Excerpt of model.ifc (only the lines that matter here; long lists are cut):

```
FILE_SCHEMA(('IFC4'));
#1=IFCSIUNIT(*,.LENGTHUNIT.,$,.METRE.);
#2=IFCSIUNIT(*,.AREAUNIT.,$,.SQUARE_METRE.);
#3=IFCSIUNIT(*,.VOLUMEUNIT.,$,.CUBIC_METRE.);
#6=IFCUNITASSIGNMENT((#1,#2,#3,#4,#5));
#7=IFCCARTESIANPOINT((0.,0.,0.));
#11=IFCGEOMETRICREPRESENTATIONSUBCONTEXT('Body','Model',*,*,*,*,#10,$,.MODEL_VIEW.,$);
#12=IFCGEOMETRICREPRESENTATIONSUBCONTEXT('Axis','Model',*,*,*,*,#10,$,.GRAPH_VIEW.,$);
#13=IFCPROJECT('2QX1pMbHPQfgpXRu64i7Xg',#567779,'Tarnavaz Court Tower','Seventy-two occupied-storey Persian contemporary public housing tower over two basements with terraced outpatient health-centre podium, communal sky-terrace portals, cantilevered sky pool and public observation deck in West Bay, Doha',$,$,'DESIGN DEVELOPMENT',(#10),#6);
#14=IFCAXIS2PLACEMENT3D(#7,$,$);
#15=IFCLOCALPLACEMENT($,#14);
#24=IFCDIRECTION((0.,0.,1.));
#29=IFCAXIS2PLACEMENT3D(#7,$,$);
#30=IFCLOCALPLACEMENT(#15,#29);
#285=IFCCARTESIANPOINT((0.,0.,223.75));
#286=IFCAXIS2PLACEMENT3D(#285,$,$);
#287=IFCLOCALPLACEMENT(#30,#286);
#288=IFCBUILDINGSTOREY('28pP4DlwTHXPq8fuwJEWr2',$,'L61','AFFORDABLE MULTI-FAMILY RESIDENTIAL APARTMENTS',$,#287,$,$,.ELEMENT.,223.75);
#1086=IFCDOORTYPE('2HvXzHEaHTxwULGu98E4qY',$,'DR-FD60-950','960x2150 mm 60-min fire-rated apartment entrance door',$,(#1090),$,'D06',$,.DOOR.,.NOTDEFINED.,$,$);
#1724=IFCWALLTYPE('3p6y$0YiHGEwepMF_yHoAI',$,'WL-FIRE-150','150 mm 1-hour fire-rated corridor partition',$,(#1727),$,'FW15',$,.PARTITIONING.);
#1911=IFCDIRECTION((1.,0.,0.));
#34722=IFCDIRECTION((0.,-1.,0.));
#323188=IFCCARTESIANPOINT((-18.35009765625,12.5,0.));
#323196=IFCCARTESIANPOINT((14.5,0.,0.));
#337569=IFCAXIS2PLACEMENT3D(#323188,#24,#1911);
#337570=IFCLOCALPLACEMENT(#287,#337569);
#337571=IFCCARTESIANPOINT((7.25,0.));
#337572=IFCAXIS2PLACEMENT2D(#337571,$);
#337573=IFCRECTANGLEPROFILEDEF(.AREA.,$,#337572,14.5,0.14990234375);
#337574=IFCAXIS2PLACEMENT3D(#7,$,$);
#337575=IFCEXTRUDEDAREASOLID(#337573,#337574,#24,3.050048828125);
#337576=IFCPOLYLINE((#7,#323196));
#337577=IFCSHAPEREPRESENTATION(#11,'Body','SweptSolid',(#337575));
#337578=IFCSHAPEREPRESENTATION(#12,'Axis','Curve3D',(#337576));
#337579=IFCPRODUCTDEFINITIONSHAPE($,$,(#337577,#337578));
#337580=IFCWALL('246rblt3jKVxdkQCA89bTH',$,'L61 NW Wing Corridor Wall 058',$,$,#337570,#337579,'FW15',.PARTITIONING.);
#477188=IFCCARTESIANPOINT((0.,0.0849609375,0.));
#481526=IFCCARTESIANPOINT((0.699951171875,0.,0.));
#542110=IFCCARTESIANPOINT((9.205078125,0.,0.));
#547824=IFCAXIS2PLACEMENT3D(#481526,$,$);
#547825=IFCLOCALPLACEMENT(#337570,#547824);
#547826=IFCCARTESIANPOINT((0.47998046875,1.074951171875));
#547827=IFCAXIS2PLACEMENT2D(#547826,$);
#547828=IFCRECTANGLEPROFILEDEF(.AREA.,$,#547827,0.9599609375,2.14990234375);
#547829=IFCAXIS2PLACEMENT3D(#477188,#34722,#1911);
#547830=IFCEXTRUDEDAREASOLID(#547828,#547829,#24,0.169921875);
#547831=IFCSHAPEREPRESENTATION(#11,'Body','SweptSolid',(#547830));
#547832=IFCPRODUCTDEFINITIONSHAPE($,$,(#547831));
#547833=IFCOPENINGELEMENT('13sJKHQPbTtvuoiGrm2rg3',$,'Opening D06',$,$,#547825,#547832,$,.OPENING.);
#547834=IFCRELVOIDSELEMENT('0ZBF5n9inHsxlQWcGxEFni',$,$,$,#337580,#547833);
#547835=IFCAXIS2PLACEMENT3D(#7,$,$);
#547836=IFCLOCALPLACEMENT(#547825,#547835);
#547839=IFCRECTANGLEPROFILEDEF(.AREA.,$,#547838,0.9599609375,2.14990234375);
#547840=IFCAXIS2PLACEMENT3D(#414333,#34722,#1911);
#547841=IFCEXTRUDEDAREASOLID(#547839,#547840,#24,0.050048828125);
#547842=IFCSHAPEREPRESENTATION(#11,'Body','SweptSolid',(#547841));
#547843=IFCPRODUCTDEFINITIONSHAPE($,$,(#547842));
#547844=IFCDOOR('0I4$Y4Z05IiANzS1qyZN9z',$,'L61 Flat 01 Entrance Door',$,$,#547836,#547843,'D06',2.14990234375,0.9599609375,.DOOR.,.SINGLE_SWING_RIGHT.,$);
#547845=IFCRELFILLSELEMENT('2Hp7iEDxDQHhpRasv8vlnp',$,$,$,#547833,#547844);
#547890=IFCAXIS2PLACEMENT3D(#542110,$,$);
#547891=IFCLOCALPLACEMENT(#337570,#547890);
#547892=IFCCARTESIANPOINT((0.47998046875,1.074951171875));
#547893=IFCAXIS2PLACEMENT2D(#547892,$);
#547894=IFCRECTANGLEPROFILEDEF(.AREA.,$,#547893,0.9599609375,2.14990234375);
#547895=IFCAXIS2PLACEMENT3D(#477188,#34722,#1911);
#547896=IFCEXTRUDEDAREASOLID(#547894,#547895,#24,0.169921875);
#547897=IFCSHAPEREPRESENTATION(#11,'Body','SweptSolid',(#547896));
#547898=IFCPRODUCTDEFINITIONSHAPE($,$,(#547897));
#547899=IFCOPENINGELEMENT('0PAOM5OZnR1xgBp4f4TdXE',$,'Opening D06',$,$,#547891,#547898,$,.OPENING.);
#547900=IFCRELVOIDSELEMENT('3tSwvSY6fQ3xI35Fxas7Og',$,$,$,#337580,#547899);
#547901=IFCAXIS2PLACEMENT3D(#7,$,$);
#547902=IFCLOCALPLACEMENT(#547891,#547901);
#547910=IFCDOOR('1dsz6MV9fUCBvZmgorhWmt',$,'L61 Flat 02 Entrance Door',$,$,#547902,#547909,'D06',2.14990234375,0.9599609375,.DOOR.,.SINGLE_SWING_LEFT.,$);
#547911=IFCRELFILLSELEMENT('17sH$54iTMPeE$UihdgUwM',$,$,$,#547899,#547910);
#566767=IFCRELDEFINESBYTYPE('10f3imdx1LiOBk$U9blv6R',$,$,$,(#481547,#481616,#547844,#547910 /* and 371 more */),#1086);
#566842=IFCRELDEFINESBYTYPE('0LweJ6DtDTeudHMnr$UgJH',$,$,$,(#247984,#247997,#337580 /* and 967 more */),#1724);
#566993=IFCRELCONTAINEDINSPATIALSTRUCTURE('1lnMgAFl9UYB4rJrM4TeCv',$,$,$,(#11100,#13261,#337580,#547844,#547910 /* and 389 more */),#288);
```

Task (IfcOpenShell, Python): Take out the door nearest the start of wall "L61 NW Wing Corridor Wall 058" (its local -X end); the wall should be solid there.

```python
import ifcopenshell
import ifcopenshell.api.feature
import ifcopenshell.api.root
import ifcopenshell.geom
import ifcopenshell.util.shape

model = ifcopenshell.open("model.ifc")
settings = ifcopenshell.geom.settings()


def volume(element):
    """Net volume in cubic metres, openings subtracted."""
    shape = ifcopenshell.geom.create_shape(settings, element)
    return ifcopenshell.util.shape.get_volume(shape.geometry)


door = model.by_guid("0I4$Y4Z05IiANzS1qyZN9z")
opening = door.FillsVoids[0].RelatingOpeningElement
wall = opening.VoidsElements[0].RelatingBuildingElement
before = volume(wall)

ifcopenshell.api.root.remove_product(model, product=door)
ifcopenshell.api.feature.remove_feature(model, feature=opening)

after = volume(wall)

print(f"wall volume {before:.3f} -> {after:.3f} m3")

model.write("model_rev.ifc")
```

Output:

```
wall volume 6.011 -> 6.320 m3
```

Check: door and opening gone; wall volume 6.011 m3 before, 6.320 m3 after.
